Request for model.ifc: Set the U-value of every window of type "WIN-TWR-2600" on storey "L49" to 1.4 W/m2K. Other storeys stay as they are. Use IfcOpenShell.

First a look at what the model holds.

```python
import ifcopenshell
import ifcopenshell.util.element

model = ifcopenshell.open("model.ifc")
print(model.schema)
storey = next(s for s in model.by_type("IfcBuildingStorey") if s.Name == "L49")
windows = [e for e in ifcopenshell.util.element.get_decomposition(storey) if e.is_a("IfcWindow")]
seen = {}
for e in windows:
    element_type = ifcopenshell.util.element.get_type(e)
    key = (element_type.Name if element_type != e and element_type else None, ifcopenshell.util.element.get_pset(e, "Pset_WindowCommon", "ThermalTransmittance"))
    seen[key] = seen.get(key, 0) + 1
for (name, value), count in sorted(seen.items(), key=str):
    print(count, "x", name, "|", value)
```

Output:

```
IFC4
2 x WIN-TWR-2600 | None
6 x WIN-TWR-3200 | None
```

```python
import ifcopenshell
import ifcopenshell.api.pset
import ifcopenshell.util.element

model = ifcopenshell.open("model.ifc")

storey = next(s for s in model.by_type("IfcBuildingStorey") if s.Name == "L49")
windows = [e for e in ifcopenshell.util.element.get_decomposition(storey) if e.is_a("IfcWindow")]

count = 0
for e in windows:
    element_type = ifcopenshell.util.element.get_type(e)
    if element_type in (None, e) or element_type.Name != "WIN-TWR-2600":
        continue
    # add_pset returns the element's existing set when there is one.
    pset = ifcopenshell.api.pset.add_pset(model, product=e, name="Pset_WindowCommon")
    ifcopenshell.api.pset.edit_pset(model, pset=pset, properties={"ThermalTransmittance": 1.4})
    count += 1

print(count, "windows updated")

model.write("model_rev.ifc")
```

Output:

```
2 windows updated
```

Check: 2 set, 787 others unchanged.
